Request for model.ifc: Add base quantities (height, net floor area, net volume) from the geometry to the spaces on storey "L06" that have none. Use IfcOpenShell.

First a look at what the model holds.

```python
import ifcopenshell
import ifcopenshell.util.element
import ifcopenshell.util.unit

model = ifcopenshell.open("model.ifc")
print(model.schema)
for unit_type in ("LENGTHUNIT", "AREAUNIT", "VOLUMEUNIT"):
    print(unit_type, ifcopenshell.util.unit.calculate_unit_scale(model, unit_type))
storey = next(s for s in model.by_type("IfcBuildingStorey") if s.Name == "L06")
spaces = [e for e in ifcopenshell.util.element.get_decomposition(storey) if e.is_a("IfcSpace")]
for e in sorted(spaces, key=lambda e: e.id()):
    print(e.id(), e.is_a(), e.Name, list(ifcopenshell.util.element.get_psets(e, qtos_only=True)), sep=" | ")
```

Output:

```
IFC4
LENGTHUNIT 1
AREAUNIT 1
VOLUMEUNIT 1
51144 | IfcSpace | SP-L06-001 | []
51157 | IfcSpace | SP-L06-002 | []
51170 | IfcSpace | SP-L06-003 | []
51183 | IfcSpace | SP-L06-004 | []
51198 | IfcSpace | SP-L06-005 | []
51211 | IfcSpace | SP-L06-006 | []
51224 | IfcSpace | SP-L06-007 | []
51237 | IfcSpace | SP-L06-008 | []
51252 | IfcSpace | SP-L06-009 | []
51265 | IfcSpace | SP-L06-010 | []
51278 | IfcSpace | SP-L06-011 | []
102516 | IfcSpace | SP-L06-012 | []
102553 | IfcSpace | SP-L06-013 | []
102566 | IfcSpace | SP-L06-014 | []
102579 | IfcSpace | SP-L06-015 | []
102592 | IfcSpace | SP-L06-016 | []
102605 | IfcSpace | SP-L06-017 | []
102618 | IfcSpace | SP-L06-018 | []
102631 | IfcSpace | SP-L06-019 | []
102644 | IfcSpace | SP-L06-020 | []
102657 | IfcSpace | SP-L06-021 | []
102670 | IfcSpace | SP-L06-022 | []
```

```python
import ifcopenshell
import ifcopenshell.api.pset
import ifcopenshell.geom
import ifcopenshell.util.element
import ifcopenshell.util.shape
import ifcopenshell.util.unit

model = ifcopenshell.open("model.ifc")
unit_scale = ifcopenshell.util.unit.calculate_unit_scale(model)
area_scale = ifcopenshell.util.unit.calculate_unit_scale(model, "AREAUNIT")
volume_scale = ifcopenshell.util.unit.calculate_unit_scale(model, "VOLUMEUNIT")
settings = ifcopenshell.geom.settings()

storey = next(s for s in model.by_type("IfcBuildingStorey") if s.Name == "L06")
spaces = [e for e in ifcopenshell.util.element.get_decomposition(storey) if e.is_a("IfcSpace")]

for e in sorted(spaces, key=lambda e: e.id()):
    if ifcopenshell.util.element.get_psets(e, qtos_only=True, should_inherit=False):
        continue
    # Geometry comes back in metres, in the element's own axes.
    shape = ifcopenshell.geom.create_shape(settings, e)
    values = {
        "Height": ifcopenshell.util.shape.get_z(shape.geometry) / unit_scale,
        "NetFloorArea": ifcopenshell.util.shape.get_footprint_area(shape.geometry) / area_scale,
        "NetVolume": ifcopenshell.util.shape.get_volume(shape.geometry) / volume_scale,
    }
    qto = ifcopenshell.api.pset.add_qto(model, product=e, name="Qto_SpaceBaseQuantities")
    ifcopenshell.api.pset.edit_qto(model, qto=qto, properties=values)
    print(e.id(), {k: round(v, 3) for k, v in values.items()})

model.write("model-out.ifc")
```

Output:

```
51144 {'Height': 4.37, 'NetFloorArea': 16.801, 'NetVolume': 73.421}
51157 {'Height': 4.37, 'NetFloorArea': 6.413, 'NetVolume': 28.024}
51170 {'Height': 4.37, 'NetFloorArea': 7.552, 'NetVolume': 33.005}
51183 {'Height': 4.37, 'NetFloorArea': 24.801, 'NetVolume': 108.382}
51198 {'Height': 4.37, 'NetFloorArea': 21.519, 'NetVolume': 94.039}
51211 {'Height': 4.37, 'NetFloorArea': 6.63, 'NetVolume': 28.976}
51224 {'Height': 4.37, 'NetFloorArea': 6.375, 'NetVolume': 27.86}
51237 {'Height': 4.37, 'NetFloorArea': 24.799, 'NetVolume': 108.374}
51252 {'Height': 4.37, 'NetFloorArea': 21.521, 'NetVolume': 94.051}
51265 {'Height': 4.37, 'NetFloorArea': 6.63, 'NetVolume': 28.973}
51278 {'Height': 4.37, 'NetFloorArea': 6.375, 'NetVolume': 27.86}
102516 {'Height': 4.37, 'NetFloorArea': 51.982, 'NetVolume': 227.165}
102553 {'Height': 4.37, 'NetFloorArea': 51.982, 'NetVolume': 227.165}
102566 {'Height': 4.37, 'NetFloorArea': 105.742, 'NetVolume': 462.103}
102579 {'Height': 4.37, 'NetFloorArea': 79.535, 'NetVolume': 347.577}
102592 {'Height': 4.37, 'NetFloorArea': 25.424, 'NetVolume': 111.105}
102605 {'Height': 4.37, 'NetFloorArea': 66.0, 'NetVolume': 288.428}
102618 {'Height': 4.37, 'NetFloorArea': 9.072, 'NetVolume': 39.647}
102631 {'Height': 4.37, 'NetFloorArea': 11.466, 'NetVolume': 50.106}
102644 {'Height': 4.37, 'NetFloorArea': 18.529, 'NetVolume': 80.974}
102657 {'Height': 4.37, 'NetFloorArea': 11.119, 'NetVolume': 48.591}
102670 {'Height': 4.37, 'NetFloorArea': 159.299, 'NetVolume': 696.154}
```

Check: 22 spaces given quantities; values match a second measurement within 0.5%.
